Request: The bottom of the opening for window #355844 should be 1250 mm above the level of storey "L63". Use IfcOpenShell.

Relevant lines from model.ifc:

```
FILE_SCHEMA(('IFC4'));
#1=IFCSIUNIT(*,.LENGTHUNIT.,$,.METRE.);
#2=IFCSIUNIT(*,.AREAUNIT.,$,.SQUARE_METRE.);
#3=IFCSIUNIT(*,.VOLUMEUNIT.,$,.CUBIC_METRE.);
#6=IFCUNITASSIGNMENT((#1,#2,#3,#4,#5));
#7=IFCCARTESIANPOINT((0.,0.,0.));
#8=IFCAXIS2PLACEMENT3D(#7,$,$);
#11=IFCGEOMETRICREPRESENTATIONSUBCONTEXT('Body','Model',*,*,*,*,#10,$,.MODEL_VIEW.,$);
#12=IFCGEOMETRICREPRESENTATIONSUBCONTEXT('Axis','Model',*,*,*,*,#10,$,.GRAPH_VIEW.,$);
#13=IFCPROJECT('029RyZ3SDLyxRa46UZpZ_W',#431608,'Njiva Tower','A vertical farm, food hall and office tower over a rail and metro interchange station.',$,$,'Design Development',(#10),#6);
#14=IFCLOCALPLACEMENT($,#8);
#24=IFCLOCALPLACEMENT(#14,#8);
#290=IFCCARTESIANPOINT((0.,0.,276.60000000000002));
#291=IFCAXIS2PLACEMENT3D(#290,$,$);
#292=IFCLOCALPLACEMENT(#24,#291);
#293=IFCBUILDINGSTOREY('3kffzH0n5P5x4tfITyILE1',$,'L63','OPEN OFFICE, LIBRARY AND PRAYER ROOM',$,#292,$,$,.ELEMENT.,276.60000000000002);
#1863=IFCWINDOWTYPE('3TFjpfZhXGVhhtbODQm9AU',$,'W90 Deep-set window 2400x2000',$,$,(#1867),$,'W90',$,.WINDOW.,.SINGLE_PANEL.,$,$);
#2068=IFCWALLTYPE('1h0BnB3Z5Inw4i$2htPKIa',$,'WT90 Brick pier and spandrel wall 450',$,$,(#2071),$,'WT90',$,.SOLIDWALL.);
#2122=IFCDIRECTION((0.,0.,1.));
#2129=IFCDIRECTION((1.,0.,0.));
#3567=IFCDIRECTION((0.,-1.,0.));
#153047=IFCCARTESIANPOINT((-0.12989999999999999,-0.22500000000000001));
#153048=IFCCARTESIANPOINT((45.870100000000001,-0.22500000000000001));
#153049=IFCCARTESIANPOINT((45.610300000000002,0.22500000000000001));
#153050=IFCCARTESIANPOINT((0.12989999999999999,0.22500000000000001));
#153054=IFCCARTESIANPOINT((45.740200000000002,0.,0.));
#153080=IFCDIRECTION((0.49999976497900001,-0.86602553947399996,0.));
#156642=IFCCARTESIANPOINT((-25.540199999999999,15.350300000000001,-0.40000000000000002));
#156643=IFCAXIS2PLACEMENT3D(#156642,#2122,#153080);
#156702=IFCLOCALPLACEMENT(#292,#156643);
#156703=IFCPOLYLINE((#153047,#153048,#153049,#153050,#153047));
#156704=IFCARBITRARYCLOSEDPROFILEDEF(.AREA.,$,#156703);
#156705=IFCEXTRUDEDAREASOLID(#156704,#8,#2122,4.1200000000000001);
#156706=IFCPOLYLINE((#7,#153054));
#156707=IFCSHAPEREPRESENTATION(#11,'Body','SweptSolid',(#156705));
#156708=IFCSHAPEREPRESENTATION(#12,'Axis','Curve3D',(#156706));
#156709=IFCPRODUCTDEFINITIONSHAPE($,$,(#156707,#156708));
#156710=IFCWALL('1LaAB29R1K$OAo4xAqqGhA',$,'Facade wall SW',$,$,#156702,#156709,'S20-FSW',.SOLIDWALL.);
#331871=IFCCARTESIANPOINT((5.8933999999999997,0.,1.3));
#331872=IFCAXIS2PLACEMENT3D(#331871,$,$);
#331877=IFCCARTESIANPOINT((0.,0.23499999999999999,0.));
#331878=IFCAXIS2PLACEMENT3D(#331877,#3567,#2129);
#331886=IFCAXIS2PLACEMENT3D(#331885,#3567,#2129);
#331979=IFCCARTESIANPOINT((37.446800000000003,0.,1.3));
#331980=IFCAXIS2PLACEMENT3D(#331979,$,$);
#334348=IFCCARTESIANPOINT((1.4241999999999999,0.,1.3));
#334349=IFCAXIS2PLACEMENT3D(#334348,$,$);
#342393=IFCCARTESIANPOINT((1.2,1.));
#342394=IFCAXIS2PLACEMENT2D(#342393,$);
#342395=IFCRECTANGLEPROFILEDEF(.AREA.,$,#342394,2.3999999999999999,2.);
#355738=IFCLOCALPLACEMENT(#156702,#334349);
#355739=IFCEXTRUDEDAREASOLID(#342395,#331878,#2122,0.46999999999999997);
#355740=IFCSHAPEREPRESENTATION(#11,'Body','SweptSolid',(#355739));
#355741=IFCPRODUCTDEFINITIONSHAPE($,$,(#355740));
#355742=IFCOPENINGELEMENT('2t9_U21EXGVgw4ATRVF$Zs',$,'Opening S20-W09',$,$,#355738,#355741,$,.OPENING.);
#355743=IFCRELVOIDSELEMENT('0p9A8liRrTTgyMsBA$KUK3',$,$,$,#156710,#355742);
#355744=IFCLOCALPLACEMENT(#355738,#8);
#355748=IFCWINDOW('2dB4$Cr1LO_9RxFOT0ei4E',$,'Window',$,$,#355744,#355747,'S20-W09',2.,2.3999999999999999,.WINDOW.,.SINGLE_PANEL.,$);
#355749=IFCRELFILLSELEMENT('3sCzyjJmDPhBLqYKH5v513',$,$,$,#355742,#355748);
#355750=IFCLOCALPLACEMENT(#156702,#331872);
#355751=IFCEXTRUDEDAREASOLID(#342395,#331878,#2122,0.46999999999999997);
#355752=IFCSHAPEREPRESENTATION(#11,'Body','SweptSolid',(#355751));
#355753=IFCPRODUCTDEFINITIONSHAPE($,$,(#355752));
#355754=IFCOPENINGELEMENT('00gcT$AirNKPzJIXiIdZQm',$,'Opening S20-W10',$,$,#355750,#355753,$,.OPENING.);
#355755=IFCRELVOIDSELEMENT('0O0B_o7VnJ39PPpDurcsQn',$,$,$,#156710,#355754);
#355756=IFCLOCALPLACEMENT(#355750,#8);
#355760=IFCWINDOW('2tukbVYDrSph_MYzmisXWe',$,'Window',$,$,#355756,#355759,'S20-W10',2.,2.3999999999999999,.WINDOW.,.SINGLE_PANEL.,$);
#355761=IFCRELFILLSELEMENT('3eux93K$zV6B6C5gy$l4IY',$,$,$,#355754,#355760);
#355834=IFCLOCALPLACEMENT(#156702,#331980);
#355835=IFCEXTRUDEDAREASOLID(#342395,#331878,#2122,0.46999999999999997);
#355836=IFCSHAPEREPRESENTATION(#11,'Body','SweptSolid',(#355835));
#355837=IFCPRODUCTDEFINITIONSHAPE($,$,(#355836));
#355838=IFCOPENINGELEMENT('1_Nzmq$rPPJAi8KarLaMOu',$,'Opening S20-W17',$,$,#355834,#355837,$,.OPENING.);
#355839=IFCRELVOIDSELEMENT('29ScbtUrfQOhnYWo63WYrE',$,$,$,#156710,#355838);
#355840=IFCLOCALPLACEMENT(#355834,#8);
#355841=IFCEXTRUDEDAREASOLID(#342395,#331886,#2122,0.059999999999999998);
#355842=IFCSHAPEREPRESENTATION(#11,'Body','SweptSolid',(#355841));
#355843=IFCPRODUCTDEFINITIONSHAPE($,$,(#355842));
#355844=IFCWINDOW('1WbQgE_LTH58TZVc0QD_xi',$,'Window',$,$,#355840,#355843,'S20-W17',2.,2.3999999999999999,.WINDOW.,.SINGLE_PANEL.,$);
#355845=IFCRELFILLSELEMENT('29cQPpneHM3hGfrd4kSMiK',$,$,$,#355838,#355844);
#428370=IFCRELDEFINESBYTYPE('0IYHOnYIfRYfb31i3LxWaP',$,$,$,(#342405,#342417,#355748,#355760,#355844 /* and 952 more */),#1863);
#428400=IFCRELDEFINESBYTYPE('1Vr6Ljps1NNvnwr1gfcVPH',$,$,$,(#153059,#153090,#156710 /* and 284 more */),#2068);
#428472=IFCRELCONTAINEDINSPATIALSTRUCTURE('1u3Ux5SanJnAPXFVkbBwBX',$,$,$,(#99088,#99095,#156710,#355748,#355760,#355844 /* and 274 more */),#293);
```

```python
import numpy as np
import ifcopenshell
import ifcopenshell.api.geometry
import ifcopenshell.geom
import ifcopenshell.util.element
import ifcopenshell.util.placement
import ifcopenshell.util.shape
import ifcopenshell.util.unit

model = ifcopenshell.open("model.ifc")
unit_scale = ifcopenshell.util.unit.calculate_unit_scale(model)

window = model.by_guid("1WbQgE_LTH58TZVc0QD_xi")
opening = window.FillsVoids[0].RelatingOpeningElement
storey = ifcopenshell.util.element.get_container(window, ifc_class="IfcBuildingStorey")
level = ifcopenshell.util.placement.get_local_placement(storey.ObjectPlacement)[2, 3]

# The opening's origin need not be at the sill, so measure its lowest point.
shape = ifcopenshell.geom.create_shape(ifcopenshell.geom.settings(), opening)
bottom = ifcopenshell.util.shape.get_shape_bottom_elevation(shape, shape.geometry) / unit_scale
dz = level + 1.25 / unit_scale - bottom

shift = np.array([0.0, 0.0, dz])
# The window is placed relative to its opening, so it follows when the opening moves.
matrix = ifcopenshell.util.placement.get_local_placement(opening.ObjectPlacement)
matrix[:3, 3] += shift
ifcopenshell.api.geometry.edit_object_placement(
    model, product=opening, matrix=matrix, is_si=False, should_transform_children=True
)

print(f"moved by {dz * unit_scale:+.3f} m")

model.write("model_updated.ifc")
```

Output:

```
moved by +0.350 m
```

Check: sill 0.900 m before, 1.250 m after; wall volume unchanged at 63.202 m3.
